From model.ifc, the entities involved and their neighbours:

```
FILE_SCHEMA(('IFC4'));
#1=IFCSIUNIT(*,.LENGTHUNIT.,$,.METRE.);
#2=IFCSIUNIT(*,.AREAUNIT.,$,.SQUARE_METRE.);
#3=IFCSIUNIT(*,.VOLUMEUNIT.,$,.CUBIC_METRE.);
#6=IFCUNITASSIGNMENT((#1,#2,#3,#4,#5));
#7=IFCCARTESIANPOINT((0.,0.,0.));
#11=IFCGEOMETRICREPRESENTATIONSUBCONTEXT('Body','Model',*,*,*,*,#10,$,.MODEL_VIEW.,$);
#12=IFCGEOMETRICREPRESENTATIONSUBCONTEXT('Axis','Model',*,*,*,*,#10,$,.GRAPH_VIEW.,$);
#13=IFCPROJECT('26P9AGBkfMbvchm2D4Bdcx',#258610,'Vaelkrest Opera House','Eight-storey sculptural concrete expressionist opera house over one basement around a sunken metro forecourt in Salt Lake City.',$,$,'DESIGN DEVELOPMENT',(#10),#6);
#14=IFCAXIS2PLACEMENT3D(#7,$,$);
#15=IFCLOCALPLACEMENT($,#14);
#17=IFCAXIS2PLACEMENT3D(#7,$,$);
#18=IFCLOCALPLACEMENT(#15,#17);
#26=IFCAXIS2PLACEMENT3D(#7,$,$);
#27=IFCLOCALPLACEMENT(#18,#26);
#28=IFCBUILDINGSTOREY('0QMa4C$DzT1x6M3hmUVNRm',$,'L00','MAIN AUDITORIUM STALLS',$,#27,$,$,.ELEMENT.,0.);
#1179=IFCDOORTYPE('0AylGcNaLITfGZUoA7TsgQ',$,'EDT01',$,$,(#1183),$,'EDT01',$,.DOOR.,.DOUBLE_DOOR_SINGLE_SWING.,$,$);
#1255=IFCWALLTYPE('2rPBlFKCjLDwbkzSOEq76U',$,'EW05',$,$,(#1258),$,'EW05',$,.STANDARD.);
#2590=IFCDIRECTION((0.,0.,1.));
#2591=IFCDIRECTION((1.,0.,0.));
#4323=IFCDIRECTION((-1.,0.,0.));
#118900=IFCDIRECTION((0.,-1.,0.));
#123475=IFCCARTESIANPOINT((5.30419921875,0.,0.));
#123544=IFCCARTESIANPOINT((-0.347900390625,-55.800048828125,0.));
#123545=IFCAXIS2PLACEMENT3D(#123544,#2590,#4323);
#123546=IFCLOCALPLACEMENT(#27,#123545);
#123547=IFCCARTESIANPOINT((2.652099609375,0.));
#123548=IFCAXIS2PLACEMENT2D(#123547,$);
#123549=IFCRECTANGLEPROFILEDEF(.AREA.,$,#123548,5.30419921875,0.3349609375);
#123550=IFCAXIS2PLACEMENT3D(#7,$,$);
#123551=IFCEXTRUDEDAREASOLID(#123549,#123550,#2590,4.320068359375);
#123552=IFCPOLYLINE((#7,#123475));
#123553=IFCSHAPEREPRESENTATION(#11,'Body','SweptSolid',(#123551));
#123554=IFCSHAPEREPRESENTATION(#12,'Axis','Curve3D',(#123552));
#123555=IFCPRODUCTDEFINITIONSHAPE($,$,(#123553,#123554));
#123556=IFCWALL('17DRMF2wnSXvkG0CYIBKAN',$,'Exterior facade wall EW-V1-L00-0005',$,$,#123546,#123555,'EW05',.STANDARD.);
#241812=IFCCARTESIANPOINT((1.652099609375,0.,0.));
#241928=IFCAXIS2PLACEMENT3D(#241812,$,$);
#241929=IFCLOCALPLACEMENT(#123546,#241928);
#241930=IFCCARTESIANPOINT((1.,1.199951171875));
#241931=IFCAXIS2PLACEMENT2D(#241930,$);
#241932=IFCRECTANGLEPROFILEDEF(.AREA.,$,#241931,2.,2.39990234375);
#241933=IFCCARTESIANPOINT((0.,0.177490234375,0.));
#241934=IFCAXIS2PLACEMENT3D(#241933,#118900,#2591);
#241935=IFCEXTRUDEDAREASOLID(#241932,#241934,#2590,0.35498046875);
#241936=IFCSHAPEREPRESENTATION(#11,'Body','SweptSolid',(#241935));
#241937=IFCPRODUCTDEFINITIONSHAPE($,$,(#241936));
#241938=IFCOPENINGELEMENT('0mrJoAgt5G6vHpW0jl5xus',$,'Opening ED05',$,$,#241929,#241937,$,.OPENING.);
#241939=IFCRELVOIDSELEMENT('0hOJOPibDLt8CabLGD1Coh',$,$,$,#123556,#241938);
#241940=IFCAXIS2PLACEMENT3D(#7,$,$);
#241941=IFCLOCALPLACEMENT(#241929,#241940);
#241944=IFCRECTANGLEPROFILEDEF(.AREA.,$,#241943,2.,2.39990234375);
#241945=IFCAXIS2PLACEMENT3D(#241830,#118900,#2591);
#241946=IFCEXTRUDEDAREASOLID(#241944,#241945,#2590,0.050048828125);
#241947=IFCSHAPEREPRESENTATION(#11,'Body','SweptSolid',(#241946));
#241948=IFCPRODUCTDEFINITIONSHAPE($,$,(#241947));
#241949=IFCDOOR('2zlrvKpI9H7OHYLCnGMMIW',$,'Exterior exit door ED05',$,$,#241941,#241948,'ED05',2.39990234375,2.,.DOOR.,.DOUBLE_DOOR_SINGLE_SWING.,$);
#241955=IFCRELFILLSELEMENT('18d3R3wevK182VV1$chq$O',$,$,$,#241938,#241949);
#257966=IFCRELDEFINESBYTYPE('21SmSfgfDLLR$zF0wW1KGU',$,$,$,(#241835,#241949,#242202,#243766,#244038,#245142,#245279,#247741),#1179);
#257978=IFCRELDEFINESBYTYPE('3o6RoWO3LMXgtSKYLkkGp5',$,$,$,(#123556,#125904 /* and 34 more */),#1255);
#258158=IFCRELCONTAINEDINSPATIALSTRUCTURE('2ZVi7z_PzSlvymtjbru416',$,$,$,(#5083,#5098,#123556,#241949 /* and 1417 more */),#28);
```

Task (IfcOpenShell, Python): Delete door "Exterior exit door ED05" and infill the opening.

```python
import ifcopenshell
import ifcopenshell.api.feature
import ifcopenshell.api.root
import ifcopenshell.geom
import ifcopenshell.util.shape

model = ifcopenshell.open("model.ifc")
settings = ifcopenshell.geom.settings()


def volume(element):
    """Net volume in cubic metres, openings subtracted."""
    shape = ifcopenshell.geom.create_shape(settings, element)
    return ifcopenshell.util.shape.get_volume(shape.geometry)


door = model.by_id(241949)
opening = door.FillsVoids[0].RelatingOpeningElement
wall = opening.VoidsElements[0].RelatingBuildingElement
before = volume(wall)

ifcopenshell.api.root.remove_product(model, product=door)
ifcopenshell.api.feature.remove_feature(model, feature=opening)

after = volume(wall)

print(f"wall volume {before:.3f} -> {after:.3f} m3")

model.write("model-out.ifc")
```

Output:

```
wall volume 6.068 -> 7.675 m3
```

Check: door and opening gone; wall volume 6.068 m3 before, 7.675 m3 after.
